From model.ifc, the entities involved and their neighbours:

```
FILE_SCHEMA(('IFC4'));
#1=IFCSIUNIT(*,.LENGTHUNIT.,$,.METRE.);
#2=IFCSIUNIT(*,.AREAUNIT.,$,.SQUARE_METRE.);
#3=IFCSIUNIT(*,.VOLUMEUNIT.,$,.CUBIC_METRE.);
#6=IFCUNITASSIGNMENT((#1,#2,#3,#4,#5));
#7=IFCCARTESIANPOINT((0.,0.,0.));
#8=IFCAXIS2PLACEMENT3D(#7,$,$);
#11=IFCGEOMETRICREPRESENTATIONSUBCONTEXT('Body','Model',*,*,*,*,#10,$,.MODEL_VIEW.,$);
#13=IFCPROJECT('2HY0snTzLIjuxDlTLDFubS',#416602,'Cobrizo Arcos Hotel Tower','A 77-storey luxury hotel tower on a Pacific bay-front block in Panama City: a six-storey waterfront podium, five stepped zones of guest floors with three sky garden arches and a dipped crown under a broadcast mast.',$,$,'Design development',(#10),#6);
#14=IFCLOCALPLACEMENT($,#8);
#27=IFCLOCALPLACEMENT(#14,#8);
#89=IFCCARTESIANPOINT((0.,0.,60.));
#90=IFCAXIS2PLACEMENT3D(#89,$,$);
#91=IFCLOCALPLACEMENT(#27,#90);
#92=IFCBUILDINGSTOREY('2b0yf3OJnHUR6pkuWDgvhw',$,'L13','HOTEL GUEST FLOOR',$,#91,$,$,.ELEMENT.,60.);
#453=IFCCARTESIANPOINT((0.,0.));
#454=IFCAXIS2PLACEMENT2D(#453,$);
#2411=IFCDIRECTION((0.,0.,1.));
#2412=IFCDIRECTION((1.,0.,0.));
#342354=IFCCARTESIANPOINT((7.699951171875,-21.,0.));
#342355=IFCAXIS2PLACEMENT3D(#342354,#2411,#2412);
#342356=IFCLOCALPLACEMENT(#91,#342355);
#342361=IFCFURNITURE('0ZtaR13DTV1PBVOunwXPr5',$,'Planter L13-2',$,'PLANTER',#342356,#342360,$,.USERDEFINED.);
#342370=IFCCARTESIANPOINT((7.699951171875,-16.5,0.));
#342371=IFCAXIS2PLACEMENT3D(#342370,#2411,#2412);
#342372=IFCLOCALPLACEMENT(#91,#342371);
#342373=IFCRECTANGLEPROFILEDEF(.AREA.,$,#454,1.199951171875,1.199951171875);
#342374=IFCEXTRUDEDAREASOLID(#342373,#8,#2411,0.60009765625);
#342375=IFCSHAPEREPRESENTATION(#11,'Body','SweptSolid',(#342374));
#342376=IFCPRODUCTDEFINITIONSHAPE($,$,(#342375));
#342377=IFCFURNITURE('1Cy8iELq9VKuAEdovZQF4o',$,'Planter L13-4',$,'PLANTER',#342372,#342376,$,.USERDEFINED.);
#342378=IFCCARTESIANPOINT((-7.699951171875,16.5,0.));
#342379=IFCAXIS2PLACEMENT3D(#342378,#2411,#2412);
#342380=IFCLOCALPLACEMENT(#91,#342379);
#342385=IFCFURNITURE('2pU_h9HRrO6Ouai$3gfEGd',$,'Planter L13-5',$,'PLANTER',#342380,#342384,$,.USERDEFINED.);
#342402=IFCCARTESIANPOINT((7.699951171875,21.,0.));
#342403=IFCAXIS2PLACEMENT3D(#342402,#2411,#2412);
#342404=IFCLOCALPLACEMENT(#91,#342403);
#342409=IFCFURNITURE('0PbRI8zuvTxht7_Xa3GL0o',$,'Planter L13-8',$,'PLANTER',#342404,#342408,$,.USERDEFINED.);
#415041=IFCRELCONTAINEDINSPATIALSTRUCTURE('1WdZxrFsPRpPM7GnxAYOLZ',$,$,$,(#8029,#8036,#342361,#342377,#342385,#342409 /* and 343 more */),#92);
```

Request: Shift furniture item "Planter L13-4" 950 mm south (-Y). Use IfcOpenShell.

```python
import ifcopenshell
import ifcopenshell.api.geometry
import ifcopenshell.util.placement
import ifcopenshell.util.unit

model = ifcopenshell.open("model.ifc")
unit_scale = ifcopenshell.util.unit.calculate_unit_scale(model)

item = model.by_id(342377)
matrix = ifcopenshell.util.placement.get_local_placement(item.ObjectPlacement)
matrix[1, 3] -= 0.95 / unit_scale
ifcopenshell.api.geometry.edit_object_placement(model, product=item, matrix=matrix, is_si=False)

print(ifcopenshell.util.placement.get_local_placement(item.ObjectPlacement).round(3) + 0.0)

model.write("model_updated.ifc")
```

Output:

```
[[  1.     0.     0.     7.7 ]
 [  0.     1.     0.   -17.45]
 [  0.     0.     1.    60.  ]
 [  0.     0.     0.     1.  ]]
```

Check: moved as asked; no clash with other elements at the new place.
